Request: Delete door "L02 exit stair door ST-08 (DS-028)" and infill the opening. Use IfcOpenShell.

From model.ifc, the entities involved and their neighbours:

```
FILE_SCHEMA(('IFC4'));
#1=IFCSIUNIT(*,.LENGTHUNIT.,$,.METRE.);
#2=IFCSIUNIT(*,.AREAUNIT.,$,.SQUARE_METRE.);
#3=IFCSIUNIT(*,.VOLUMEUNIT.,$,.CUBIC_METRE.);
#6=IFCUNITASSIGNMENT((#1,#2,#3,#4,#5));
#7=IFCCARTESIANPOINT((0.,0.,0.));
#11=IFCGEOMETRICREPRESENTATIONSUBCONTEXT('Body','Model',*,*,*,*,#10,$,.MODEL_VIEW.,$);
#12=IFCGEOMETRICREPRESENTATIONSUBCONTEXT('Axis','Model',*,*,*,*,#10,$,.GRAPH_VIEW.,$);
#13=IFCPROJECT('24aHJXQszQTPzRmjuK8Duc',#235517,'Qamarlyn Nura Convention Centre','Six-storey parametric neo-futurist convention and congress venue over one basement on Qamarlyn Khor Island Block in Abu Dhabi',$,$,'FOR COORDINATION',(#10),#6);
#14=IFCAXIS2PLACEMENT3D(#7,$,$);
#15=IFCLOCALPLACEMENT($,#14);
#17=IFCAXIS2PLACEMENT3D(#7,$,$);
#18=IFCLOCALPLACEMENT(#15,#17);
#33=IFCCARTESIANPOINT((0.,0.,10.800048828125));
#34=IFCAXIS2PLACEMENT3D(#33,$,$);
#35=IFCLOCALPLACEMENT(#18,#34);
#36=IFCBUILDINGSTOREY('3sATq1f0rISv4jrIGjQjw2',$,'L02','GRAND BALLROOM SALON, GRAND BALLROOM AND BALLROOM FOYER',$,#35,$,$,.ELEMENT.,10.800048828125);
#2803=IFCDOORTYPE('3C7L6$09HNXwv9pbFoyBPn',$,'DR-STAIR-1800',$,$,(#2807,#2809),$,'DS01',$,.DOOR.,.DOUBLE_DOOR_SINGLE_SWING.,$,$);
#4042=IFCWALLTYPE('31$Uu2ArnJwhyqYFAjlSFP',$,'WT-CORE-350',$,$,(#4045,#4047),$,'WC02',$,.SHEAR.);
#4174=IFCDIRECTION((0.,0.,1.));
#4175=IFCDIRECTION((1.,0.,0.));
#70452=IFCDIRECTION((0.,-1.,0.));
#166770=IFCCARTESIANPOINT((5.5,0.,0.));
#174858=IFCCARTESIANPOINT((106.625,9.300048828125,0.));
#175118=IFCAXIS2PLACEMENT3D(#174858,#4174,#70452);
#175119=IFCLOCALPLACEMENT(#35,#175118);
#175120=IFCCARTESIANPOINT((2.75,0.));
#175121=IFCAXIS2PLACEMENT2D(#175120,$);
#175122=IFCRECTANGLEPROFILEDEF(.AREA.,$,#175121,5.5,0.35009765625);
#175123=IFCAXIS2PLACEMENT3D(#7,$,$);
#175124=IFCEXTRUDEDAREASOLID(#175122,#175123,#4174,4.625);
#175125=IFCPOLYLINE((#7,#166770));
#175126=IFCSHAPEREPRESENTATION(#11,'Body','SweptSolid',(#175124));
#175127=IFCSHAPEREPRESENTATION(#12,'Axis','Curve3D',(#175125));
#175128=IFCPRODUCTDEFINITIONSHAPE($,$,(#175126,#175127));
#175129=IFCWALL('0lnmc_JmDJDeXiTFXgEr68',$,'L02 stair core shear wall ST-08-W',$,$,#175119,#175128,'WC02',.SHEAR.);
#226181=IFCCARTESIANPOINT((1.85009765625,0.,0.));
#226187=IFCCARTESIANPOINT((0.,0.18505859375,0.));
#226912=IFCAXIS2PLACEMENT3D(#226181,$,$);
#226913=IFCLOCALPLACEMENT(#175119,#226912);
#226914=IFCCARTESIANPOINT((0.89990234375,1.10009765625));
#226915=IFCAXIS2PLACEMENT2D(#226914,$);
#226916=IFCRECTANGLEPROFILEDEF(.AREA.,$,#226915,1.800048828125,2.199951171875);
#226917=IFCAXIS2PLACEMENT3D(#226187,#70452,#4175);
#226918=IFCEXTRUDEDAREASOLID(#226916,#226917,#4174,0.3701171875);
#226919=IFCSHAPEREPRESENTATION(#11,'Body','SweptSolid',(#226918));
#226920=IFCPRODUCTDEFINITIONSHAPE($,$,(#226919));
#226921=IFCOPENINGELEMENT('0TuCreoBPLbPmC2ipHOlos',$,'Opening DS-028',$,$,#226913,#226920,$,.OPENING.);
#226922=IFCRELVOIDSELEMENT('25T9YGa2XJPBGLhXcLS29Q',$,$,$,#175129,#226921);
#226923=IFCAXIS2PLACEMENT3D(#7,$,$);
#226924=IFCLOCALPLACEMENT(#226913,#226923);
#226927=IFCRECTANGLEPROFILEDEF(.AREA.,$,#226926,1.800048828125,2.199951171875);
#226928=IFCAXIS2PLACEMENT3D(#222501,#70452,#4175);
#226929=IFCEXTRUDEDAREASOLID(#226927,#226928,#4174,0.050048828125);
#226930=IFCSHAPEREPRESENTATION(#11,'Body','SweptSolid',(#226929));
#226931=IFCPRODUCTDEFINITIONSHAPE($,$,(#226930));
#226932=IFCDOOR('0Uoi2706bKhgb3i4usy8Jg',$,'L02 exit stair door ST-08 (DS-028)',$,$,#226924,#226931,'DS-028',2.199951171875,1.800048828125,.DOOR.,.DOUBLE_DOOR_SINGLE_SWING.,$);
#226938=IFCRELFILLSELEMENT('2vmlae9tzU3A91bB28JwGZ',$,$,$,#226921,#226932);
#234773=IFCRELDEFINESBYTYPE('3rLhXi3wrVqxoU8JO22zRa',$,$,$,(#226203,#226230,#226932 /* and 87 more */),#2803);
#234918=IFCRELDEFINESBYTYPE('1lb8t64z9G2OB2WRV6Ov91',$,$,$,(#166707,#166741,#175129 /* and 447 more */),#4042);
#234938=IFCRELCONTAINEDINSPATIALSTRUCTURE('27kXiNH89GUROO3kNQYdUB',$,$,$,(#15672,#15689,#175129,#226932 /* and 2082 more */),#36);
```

```python
import ifcopenshell
import ifcopenshell.api.feature
import ifcopenshell.api.root
import ifcopenshell.geom
import ifcopenshell.util.shape

model = ifcopenshell.open("model.ifc")
settings = ifcopenshell.geom.settings()


def volume(element):
    """Net volume in cubic metres, openings subtracted."""
    shape = ifcopenshell.geom.create_shape(settings, element)
    return ifcopenshell.util.shape.get_volume(shape.geometry)


door = model.by_id(226932)
opening = door.FillsVoids[0].RelatingOpeningElement
wall = opening.VoidsElements[0].RelatingBuildingElement
before = volume(wall)

ifcopenshell.api.root.remove_product(model, product=door)
ifcopenshell.api.feature.remove_feature(model, feature=opening)

after = volume(wall)

print(f"wall volume {before:.3f} -> {after:.3f} m3")

model.write("model_updated.ifc")
```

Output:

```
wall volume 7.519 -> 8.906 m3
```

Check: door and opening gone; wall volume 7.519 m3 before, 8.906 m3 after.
